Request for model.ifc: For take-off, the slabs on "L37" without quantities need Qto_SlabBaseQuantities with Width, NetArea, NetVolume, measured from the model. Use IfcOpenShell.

First a look at what the model holds.

```python
import ifcopenshell
import ifcopenshell.util.element
import ifcopenshell.util.unit

model = ifcopenshell.open("model.ifc")
print(model.schema)
for unit_type in ("LENGTHUNIT", "AREAUNIT", "VOLUMEUNIT"):
    print(unit_type, ifcopenshell.util.unit.calculate_unit_scale(model, unit_type))
storey = next(s for s in model.by_type("IfcBuildingStorey") if s.Name == "L37")
slabs = [e for e in ifcopenshell.util.element.get_decomposition(storey) if e.is_a("IfcSlab")]
for e in sorted(slabs, key=lambda e: e.id()):
    print(e.id(), e.is_a(), e.Name, list(ifcopenshell.util.element.get_psets(e, qtos_only=True)), sep=" | ")
```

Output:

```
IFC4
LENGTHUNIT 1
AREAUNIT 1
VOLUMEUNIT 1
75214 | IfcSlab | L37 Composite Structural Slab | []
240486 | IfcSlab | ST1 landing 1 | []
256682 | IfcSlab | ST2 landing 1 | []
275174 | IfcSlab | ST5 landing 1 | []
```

```python
import ifcopenshell
import ifcopenshell.api.pset
import ifcopenshell.geom
import ifcopenshell.util.element
import ifcopenshell.util.shape
import ifcopenshell.util.unit

model = ifcopenshell.open("model.ifc")
unit_scale = ifcopenshell.util.unit.calculate_unit_scale(model)
area_scale = ifcopenshell.util.unit.calculate_unit_scale(model, "AREAUNIT")
volume_scale = ifcopenshell.util.unit.calculate_unit_scale(model, "VOLUMEUNIT")
settings = ifcopenshell.geom.settings()

storey = next(s for s in model.by_type("IfcBuildingStorey") if s.Name == "L37")
slabs = [e for e in ifcopenshell.util.element.get_decomposition(storey) if e.is_a("IfcSlab")]

for e in sorted(slabs, key=lambda e: e.id()):
    if ifcopenshell.util.element.get_psets(e, qtos_only=True, should_inherit=False):
        continue
    # Geometry comes back in metres, in the element's own axes.
    shape = ifcopenshell.geom.create_shape(settings, e)
    values = {
        "Width": ifcopenshell.util.shape.get_z(shape.geometry) / unit_scale,
        "NetArea": ifcopenshell.util.shape.get_footprint_area(shape.geometry) / area_scale,
        "NetVolume": ifcopenshell.util.shape.get_volume(shape.geometry) / volume_scale,
    }
    qto = ifcopenshell.api.pset.add_qto(model, product=e, name="Qto_SlabBaseQuantities")
    ifcopenshell.api.pset.edit_qto(model, qto=qto, properties=values)
    print(e.id(), {k: round(v, 3) for k, v in values.items()})

model.write("model_updated.ifc")
```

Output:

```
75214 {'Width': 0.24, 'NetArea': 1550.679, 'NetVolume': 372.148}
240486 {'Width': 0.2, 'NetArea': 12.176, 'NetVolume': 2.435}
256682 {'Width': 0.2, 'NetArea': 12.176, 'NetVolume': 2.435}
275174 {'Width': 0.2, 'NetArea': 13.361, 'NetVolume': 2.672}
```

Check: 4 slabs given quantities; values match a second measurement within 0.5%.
